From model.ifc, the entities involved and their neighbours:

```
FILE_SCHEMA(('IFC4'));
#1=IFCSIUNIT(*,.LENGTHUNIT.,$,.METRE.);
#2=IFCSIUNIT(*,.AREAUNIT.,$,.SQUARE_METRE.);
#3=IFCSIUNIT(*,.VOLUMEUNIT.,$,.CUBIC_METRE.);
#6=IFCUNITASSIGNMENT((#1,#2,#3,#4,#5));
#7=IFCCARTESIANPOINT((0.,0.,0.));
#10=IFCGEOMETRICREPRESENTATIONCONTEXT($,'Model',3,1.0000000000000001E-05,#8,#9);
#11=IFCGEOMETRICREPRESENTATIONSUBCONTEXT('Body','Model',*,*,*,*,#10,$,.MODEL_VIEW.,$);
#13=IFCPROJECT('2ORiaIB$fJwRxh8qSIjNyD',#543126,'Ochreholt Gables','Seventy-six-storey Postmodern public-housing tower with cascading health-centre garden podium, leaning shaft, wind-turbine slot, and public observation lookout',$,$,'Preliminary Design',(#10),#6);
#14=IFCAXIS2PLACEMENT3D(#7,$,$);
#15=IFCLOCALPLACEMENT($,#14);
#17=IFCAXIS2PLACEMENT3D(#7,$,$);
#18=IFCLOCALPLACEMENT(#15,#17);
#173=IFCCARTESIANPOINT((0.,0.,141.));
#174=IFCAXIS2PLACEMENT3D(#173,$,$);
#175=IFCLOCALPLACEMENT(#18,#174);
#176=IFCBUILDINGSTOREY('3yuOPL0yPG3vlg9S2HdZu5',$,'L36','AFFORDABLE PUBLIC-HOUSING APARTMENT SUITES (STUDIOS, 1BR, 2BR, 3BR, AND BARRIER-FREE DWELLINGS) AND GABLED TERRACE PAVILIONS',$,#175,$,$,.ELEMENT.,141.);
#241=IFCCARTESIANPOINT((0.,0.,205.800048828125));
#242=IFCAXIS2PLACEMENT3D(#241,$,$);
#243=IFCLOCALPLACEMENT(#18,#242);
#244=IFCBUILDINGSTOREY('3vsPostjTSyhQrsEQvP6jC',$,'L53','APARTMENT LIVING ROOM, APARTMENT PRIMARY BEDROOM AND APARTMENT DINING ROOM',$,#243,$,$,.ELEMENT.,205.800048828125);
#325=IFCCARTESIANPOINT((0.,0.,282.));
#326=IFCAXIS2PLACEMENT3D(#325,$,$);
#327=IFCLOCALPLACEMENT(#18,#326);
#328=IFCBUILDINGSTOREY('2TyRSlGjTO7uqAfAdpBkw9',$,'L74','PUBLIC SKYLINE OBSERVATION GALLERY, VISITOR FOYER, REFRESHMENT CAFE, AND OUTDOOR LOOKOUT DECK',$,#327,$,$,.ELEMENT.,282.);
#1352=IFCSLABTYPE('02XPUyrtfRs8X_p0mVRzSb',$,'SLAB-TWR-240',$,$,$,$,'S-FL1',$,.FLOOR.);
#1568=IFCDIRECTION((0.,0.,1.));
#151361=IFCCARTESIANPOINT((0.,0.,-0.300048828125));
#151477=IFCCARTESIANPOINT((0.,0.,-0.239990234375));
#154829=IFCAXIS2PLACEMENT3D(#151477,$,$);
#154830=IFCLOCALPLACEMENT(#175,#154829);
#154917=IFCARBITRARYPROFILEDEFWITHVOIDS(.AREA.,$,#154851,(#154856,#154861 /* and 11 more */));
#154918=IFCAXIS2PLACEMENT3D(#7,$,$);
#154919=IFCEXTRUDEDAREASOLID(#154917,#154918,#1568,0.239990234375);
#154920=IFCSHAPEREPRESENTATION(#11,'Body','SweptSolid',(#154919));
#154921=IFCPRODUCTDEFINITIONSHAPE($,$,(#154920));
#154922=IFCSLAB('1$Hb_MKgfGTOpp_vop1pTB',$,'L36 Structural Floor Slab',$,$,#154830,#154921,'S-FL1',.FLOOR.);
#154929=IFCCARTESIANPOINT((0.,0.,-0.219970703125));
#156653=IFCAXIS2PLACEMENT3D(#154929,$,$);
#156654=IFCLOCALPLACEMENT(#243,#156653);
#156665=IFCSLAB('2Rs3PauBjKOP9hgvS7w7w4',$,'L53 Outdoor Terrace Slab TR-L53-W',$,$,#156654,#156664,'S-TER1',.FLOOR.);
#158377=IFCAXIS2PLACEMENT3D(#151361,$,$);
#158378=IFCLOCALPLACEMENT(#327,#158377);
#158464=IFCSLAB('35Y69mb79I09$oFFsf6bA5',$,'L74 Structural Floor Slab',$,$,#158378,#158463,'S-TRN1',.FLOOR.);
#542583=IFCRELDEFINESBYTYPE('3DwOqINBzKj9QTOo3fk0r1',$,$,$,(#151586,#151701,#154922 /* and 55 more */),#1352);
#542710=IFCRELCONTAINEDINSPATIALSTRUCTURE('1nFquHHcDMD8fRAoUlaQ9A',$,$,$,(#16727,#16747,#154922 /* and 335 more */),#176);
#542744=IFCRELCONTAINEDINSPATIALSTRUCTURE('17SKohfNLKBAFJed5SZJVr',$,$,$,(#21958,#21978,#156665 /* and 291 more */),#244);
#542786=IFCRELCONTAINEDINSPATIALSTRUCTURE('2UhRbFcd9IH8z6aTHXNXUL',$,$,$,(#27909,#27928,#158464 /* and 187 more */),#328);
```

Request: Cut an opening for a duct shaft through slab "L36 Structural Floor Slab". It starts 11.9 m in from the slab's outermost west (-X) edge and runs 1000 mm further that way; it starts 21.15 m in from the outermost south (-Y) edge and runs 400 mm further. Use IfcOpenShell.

```python
import numpy as np
import ifcopenshell
import ifcopenshell.api.feature
import ifcopenshell.api.geometry
import ifcopenshell.api.root
import ifcopenshell.geom
import ifcopenshell.util.placement
import ifcopenshell.util.representation
import ifcopenshell.util.shape
import ifcopenshell.util.unit

model = ifcopenshell.open("model.ifc")
unit_scale = ifcopenshell.util.unit.calculate_unit_scale(model)
settings = ifcopenshell.geom.settings()


def volume(element):
    """Net volume in cubic metres, openings subtracted."""
    shape = ifcopenshell.geom.create_shape(settings, element)
    return ifcopenshell.util.shape.get_volume(shape.geometry)


slab = model.by_guid("1$Hb_MKgfGTOpp_vop1pTB")
before = volume(slab)

# Extent in the slab's own axes, in metres. The edges named are its -X and -Y sides.
slab_shape = ifcopenshell.geom.create_shape(settings, slab)
vertices = ifcopenshell.util.shape.get_vertices(slab_shape.geometry)
x_min, y_min, bottom = vertices.min(axis=0)
top = vertices[:, 2].max()

opening = ifcopenshell.api.root.create_entity(model, ifc_class="IfcOpeningElement", name="Duct shaft opening", predefined_type="OPENING")
context = ifcopenshell.util.representation.get_context(model, "Model", "Body", "MODEL_VIEW")
width, depth = 1, 0.4
outline = [(0.0, 0.0), (width, 0.0), (width, depth), (0.0, depth), (0.0, 0.0)]
# Overshoot both faces by 50 mm so the cut is clean.
shape = ifcopenshell.api.geometry.add_slab_representation(
    model, context=context, depth=top - bottom + 0.1, polyline=outline
)
ifcopenshell.api.geometry.assign_representation(model, product=opening, representation=shape)

matrix = ifcopenshell.util.placement.get_local_placement(slab.ObjectPlacement)
matrix[:, 3] = matrix @ np.append(np.array([x_min + 11.9, y_min + 21.15, bottom - 0.05]) / unit_scale, 1.0)
ifcopenshell.api.geometry.edit_object_placement(model, product=opening, matrix=matrix, is_si=False)
ifcopenshell.api.feature.add_feature(model, feature=opening, element=slab)

after = volume(slab)

print(f"slab volume {before:.3f} -> {after:.3f} m3")

model.write("model_edited.ifc")
```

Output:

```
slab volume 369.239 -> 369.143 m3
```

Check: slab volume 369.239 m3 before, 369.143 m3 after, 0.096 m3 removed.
